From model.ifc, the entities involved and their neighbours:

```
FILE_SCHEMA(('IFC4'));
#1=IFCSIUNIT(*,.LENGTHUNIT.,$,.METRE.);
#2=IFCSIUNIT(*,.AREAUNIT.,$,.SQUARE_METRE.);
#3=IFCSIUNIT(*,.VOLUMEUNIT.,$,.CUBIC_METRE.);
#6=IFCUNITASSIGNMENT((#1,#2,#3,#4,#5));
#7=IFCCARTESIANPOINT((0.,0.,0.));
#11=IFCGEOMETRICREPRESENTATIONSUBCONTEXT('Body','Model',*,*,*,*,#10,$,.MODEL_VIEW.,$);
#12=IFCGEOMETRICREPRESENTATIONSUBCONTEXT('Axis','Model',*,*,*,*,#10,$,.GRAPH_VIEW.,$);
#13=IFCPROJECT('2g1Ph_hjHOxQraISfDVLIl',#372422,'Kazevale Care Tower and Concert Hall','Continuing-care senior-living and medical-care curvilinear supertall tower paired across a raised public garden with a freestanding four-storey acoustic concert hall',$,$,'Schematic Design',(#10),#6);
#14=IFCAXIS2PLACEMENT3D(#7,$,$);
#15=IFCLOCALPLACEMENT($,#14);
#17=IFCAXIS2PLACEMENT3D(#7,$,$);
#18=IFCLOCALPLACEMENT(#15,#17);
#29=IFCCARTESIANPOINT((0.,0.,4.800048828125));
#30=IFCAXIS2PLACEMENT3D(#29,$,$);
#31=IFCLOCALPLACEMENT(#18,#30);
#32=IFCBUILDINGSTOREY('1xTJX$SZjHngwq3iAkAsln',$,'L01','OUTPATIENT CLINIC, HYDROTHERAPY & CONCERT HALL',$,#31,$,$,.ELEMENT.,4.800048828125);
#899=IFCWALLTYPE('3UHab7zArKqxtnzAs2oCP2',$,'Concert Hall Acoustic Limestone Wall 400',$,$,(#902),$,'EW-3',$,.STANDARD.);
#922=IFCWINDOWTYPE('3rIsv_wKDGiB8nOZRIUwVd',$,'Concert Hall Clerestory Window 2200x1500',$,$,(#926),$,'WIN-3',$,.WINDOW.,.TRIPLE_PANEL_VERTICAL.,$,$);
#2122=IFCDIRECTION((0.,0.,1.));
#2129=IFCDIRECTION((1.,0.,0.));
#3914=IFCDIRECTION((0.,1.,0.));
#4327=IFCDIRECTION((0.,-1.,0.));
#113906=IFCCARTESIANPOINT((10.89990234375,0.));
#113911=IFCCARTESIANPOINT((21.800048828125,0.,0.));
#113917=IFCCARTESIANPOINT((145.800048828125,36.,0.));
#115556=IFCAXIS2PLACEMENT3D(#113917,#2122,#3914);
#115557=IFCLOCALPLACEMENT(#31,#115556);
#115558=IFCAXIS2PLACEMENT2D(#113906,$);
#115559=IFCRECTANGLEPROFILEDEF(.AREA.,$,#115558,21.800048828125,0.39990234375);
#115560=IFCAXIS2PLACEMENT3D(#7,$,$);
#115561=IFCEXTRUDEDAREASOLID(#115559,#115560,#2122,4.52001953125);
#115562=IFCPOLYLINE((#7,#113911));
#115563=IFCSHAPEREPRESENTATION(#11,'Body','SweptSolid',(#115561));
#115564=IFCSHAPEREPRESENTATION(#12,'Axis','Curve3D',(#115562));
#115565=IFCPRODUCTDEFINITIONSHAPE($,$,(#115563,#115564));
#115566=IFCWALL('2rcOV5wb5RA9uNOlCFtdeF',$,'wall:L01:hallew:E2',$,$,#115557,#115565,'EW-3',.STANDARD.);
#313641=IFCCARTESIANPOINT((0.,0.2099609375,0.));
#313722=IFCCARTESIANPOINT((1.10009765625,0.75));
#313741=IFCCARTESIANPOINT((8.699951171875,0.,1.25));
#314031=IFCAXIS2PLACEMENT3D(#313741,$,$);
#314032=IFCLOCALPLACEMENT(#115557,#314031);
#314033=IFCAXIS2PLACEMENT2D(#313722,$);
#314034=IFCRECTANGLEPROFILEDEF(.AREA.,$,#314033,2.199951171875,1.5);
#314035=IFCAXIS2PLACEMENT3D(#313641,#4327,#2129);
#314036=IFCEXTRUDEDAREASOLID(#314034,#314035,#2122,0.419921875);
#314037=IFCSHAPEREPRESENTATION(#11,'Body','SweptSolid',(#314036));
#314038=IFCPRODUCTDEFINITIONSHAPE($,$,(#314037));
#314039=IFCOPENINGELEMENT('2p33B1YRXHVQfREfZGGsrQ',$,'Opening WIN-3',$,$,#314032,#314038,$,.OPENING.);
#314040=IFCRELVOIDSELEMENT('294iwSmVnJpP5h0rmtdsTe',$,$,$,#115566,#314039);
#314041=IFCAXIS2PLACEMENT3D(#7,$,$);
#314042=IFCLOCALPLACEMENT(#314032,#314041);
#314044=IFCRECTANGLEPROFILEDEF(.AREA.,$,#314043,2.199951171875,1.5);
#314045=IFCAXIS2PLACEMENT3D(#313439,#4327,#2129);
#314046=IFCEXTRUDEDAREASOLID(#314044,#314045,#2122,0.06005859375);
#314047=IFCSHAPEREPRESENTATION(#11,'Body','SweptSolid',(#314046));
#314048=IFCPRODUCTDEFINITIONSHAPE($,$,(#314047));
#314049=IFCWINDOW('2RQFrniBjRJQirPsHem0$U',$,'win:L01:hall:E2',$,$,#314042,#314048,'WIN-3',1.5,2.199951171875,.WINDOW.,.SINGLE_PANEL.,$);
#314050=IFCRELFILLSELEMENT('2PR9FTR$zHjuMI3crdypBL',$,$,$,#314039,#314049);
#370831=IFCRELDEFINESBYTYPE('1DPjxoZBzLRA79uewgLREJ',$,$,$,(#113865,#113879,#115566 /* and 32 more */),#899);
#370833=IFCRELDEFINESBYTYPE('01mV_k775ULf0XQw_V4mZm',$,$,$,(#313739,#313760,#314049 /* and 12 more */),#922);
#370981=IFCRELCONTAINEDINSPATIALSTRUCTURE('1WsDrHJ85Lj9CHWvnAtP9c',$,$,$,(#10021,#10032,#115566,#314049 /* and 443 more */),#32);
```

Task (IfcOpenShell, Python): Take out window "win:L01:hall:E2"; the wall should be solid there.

```python
import ifcopenshell
import ifcopenshell.api.feature
import ifcopenshell.api.root
import ifcopenshell.geom
import ifcopenshell.util.shape

model = ifcopenshell.open("model.ifc")
settings = ifcopenshell.geom.settings()


def volume(element):
    """Net volume in cubic metres, openings subtracted."""
    shape = ifcopenshell.geom.create_shape(settings, element)
    return ifcopenshell.util.shape.get_volume(shape.geometry)


window = model.by_guid("2RQFrniBjRJQirPsHem0$U")
opening = window.FillsVoids[0].RelatingOpeningElement
wall = opening.VoidsElements[0].RelatingBuildingElement
before = volume(wall)

ifcopenshell.api.root.remove_product(model, product=window)
ifcopenshell.api.feature.remove_feature(model, feature=opening)

after = volume(wall)

print(f"wall volume {before:.3f} -> {after:.3f} m3")

model.write("model_rev.ifc")
```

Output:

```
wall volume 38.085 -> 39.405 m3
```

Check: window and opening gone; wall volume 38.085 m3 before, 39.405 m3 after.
